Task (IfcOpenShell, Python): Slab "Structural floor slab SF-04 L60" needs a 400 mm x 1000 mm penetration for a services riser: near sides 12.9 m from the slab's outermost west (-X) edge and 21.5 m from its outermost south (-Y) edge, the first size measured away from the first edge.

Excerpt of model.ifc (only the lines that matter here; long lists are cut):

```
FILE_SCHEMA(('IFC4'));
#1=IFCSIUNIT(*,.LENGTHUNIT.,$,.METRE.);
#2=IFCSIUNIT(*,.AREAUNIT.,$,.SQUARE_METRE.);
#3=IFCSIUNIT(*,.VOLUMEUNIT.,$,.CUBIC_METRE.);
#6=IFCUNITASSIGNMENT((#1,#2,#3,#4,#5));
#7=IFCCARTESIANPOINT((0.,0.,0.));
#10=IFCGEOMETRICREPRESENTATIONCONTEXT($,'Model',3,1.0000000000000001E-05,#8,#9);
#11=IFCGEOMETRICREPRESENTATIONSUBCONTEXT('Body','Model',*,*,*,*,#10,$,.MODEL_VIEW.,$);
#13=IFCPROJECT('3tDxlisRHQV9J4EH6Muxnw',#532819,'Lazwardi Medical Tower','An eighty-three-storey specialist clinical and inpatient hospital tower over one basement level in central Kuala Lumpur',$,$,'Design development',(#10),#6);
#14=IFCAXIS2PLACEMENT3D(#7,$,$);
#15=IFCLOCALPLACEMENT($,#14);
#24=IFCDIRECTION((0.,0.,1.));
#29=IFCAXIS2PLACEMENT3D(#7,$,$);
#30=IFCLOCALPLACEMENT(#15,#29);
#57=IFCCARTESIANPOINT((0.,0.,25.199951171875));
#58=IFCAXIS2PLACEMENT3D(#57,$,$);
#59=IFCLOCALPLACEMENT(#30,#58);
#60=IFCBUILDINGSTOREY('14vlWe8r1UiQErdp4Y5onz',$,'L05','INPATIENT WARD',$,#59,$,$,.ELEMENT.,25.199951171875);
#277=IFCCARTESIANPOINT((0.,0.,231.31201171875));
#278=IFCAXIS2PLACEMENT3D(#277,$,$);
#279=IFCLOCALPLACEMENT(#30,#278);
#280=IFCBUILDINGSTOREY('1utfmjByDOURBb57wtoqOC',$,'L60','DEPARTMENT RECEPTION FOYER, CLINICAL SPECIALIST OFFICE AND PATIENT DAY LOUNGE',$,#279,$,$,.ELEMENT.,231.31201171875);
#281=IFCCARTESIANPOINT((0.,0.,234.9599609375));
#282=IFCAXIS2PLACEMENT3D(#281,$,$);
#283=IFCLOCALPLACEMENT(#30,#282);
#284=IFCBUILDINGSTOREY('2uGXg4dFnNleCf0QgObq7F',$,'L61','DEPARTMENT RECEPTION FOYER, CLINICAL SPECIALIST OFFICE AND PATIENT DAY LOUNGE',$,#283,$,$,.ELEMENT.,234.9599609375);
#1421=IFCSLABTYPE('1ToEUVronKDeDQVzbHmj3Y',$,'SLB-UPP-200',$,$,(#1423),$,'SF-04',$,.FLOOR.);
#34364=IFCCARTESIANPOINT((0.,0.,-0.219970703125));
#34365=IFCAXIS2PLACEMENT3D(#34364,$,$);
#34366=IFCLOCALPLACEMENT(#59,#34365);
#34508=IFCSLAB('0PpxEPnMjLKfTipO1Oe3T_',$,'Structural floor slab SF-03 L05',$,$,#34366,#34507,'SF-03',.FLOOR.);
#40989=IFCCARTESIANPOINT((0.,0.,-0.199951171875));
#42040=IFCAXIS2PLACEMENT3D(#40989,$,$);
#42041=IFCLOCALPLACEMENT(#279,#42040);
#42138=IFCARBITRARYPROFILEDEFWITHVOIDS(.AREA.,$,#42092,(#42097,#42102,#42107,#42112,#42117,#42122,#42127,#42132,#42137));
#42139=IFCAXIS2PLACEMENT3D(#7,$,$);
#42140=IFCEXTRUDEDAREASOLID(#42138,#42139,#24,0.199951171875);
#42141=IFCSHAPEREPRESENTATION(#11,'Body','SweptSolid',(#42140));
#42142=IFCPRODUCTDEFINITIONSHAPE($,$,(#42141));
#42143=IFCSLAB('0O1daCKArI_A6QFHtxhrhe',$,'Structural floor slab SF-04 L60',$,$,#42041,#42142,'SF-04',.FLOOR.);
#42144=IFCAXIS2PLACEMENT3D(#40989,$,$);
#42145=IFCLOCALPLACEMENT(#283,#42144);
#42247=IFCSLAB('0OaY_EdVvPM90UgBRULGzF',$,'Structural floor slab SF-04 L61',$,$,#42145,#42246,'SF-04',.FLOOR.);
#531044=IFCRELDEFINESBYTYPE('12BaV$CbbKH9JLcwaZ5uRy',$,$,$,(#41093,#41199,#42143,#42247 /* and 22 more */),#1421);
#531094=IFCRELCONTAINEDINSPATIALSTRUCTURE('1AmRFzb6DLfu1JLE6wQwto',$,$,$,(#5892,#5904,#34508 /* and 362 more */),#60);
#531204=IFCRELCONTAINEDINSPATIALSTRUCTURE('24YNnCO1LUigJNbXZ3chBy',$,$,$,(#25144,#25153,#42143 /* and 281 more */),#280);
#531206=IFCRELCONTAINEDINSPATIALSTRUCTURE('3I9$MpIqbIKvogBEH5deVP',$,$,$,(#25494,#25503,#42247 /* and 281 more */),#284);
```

```python
import numpy as np
import ifcopenshell
import ifcopenshell.api.feature
import ifcopenshell.api.geometry
import ifcopenshell.api.root
import ifcopenshell.geom
import ifcopenshell.util.placement
import ifcopenshell.util.representation
import ifcopenshell.util.shape
import ifcopenshell.util.unit

model = ifcopenshell.open("model.ifc")
unit_scale = ifcopenshell.util.unit.calculate_unit_scale(model)
settings = ifcopenshell.geom.settings()


def volume(element):
    """Net volume in cubic metres, openings subtracted."""
    shape = ifcopenshell.geom.create_shape(settings, element)
    return ifcopenshell.util.shape.get_volume(shape.geometry)


slab = model.by_id(42143)
before = volume(slab)

# Extent in the slab's own axes, in metres. The edges named are its -X and -Y sides.
slab_shape = ifcopenshell.geom.create_shape(settings, slab)
vertices = ifcopenshell.util.shape.get_vertices(slab_shape.geometry)
x_min, y_min, bottom = vertices.min(axis=0)
top = vertices[:, 2].max()

opening = ifcopenshell.api.root.create_entity(model, ifc_class="IfcOpeningElement", name="Services riser opening", predefined_type="OPENING")
context = ifcopenshell.util.representation.get_context(model, "Model", "Body", "MODEL_VIEW")
width, depth = 0.4, 1
outline = [(0.0, 0.0), (width, 0.0), (width, depth), (0.0, depth), (0.0, 0.0)]
# Overshoot both faces by 50 mm so the cut is clean.
shape = ifcopenshell.api.geometry.add_slab_representation(
    model, context=context, depth=top - bottom + 0.1, polyline=outline
)
ifcopenshell.api.geometry.assign_representation(model, product=opening, representation=shape)

matrix = ifcopenshell.util.placement.get_local_placement(slab.ObjectPlacement)
matrix[:, 3] = matrix @ np.append(np.array([x_min + 12.9, y_min + 21.5, bottom - 0.05]) / unit_scale, 1.0)
ifcopenshell.api.geometry.edit_object_placement(model, product=opening, matrix=matrix, is_si=False)
ifcopenshell.api.feature.add_feature(model, feature=opening, element=slab)

after = volume(slab)

print(f"slab volume {before:.3f} -> {after:.3f} m3")

model.write("model_edited.ifc")
```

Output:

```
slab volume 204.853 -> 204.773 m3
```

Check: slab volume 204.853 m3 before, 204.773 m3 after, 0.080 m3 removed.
